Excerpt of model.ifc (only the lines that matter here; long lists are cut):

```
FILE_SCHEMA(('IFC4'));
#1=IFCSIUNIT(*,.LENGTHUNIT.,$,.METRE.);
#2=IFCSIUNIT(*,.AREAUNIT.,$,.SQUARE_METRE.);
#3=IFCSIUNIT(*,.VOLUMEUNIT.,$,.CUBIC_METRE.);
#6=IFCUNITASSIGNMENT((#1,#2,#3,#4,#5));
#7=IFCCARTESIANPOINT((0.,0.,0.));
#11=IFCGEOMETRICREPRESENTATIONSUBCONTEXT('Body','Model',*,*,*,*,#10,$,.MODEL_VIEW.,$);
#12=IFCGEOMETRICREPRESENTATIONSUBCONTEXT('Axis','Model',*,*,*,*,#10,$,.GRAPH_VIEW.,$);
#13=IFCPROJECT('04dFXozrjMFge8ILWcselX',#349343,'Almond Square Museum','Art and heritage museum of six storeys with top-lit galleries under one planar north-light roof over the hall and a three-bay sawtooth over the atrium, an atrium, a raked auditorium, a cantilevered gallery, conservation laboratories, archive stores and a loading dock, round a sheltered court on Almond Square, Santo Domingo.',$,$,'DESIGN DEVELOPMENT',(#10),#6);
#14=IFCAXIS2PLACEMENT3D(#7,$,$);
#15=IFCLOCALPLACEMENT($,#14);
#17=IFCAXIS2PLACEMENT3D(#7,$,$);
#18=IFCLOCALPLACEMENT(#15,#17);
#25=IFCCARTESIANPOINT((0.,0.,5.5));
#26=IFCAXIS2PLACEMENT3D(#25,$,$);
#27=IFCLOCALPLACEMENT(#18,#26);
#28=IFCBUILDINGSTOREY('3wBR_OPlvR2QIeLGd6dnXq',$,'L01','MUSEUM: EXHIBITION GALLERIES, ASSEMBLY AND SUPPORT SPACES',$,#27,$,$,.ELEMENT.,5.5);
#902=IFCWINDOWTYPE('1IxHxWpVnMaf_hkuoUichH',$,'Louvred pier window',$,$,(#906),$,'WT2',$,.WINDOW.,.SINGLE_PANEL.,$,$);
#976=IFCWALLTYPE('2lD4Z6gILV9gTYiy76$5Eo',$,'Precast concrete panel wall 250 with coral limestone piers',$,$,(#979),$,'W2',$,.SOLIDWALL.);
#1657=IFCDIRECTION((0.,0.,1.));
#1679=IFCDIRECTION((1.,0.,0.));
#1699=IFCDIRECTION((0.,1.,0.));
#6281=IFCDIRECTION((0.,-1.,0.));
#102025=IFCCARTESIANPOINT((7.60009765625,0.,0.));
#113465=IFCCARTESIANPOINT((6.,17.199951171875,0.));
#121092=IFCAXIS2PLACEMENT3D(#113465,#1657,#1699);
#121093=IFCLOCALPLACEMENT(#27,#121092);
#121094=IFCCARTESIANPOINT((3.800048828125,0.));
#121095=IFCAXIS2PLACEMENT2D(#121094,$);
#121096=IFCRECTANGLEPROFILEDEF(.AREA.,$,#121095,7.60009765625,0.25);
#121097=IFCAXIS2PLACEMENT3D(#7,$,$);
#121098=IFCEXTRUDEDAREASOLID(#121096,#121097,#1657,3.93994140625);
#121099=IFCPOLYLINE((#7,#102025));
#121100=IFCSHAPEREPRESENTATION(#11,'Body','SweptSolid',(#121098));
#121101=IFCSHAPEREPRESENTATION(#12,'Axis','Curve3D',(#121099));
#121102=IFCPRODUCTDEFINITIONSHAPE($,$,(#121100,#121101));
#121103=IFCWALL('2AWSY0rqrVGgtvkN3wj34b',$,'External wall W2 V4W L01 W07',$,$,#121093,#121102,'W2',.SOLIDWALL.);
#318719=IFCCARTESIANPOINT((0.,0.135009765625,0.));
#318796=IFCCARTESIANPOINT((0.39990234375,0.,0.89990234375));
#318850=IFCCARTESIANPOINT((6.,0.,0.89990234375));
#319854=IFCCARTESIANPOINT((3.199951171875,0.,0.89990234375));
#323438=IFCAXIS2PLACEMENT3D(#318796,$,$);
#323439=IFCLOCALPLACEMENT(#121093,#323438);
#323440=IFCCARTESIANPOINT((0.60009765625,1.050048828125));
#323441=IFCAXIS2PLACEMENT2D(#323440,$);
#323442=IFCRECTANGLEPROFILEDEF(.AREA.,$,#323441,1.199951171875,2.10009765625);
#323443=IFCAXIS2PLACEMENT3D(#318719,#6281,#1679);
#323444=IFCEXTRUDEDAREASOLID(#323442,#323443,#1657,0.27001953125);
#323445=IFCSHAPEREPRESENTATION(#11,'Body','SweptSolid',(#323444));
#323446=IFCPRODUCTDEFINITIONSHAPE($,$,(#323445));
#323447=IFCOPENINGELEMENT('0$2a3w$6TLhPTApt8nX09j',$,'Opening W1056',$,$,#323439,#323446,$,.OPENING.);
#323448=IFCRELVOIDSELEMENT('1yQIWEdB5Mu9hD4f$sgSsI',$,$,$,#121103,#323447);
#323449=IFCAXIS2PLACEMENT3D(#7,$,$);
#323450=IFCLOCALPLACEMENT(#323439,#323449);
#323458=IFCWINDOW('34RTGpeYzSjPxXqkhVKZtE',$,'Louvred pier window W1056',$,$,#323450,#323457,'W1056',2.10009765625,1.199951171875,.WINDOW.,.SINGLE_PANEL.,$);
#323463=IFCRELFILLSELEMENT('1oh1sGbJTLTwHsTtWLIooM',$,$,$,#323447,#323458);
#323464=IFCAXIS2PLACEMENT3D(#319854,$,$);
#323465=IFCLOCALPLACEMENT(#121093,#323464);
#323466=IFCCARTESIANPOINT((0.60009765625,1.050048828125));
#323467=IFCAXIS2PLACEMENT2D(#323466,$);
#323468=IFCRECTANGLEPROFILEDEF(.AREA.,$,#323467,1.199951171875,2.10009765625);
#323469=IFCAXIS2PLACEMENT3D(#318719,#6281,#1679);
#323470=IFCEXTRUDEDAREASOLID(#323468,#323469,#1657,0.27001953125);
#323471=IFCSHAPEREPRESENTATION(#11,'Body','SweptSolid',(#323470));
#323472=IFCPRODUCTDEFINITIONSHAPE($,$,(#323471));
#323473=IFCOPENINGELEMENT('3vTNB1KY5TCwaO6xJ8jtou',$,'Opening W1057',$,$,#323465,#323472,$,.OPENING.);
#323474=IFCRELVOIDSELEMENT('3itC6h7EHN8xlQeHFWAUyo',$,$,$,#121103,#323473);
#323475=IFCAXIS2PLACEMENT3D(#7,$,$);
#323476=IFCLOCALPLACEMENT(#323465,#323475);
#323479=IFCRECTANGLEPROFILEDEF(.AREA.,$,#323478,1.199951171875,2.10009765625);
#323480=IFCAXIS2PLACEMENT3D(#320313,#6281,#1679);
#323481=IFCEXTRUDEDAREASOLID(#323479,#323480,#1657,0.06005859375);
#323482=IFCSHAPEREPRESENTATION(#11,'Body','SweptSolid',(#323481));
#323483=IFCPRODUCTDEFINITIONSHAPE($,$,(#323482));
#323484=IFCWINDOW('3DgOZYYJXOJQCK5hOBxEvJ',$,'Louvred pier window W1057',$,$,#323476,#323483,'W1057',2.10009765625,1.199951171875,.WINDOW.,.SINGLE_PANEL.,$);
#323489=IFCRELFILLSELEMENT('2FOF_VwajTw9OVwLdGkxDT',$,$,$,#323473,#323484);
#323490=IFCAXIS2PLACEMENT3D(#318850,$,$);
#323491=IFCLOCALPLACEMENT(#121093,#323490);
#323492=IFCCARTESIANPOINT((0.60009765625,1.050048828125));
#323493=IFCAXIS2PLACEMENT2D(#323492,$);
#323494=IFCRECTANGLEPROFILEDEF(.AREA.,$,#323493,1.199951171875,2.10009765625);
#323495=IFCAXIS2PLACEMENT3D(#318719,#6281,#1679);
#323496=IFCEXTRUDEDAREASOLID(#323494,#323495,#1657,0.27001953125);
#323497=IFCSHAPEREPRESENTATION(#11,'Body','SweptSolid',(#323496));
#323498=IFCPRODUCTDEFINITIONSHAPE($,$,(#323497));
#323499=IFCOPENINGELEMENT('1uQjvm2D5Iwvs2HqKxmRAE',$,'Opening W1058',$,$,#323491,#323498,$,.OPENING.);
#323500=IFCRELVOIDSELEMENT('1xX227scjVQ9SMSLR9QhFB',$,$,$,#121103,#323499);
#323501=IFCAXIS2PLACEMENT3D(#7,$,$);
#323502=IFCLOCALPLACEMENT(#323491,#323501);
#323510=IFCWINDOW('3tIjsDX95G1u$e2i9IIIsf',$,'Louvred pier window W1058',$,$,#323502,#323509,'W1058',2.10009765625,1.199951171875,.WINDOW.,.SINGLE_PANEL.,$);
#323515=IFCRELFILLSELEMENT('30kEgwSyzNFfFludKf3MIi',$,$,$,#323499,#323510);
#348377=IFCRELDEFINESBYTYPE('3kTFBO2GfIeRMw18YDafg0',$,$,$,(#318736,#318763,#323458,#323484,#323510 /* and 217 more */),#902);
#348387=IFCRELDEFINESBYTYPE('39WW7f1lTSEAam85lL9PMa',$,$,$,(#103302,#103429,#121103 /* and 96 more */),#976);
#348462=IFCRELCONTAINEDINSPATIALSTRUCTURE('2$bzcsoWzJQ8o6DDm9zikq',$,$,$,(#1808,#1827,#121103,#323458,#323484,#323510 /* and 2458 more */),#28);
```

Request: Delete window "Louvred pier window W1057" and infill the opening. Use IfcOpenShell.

```python
import ifcopenshell
import ifcopenshell.api.feature
import ifcopenshell.api.root
import ifcopenshell.geom
import ifcopenshell.util.shape

model = ifcopenshell.open("model.ifc")
settings = ifcopenshell.geom.settings()


def volume(element):
    """Net volume in cubic metres, openings subtracted."""
    shape = ifcopenshell.geom.create_shape(settings, element)
    return ifcopenshell.util.shape.get_volume(shape.geometry)


window = model.by_guid("3DgOZYYJXOJQCK5hOBxEvJ")
opening = window.FillsVoids[0].RelatingOpeningElement
wall = opening.VoidsElements[0].RelatingBuildingElement
before = volume(wall)

ifcopenshell.api.root.remove_product(model, product=window)
ifcopenshell.api.feature.remove_feature(model, feature=opening)

after = volume(wall)

print(f"wall volume {before:.3f} -> {after:.3f} m3")

model.write("model_v2.ifc")
```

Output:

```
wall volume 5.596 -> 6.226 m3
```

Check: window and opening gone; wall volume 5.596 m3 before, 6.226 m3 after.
